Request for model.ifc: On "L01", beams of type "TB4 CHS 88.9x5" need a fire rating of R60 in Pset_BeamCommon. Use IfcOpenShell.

First a look at what the model holds.

```python
import ifcopenshell
import ifcopenshell.util.element

model = ifcopenshell.open("model.ifc")
print(model.schema)
storey = next(s for s in model.by_type("IfcBuildingStorey") if s.Name == "L01")
beams = [e for e in ifcopenshell.util.element.get_decomposition(storey) if e.is_a("IfcBeam")]
seen = {}
for e in beams:
    element_type = ifcopenshell.util.element.get_type(e)
    key = (element_type.Name if element_type != e and element_type else None, ifcopenshell.util.element.get_pset(e, "Pset_BeamCommon", "FireRating"))
    seen[key] = seen.get(key, 0) + 1
for (name, value), count in sorted(seen.items(), key=str):
    print(count, "x", name, "|", value)
```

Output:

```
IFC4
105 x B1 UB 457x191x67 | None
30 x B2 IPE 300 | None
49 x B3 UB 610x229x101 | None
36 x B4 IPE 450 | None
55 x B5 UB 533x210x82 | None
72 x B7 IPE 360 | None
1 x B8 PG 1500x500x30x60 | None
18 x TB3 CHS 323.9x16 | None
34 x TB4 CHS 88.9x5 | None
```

```python
import ifcopenshell
import ifcopenshell.api.pset
import ifcopenshell.util.element

model = ifcopenshell.open("model.ifc")

storey = next(s for s in model.by_type("IfcBuildingStorey") if s.Name == "L01")
beams = [e for e in ifcopenshell.util.element.get_decomposition(storey) if e.is_a("IfcBeam")]

count = 0
for e in beams:
    element_type = ifcopenshell.util.element.get_type(e)
    if element_type in (None, e) or element_type.Name != "TB4 CHS 88.9x5":
        continue
    # add_pset returns the element's existing set when there is one.
    pset = ifcopenshell.api.pset.add_pset(model, product=e, name="Pset_BeamCommon")
    ifcopenshell.api.pset.edit_pset(model, pset=pset, properties={"FireRating": "R60"})
    count += 1

print(count, "beams updated")

model.write("model_updated.ifc")
```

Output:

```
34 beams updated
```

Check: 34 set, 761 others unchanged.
